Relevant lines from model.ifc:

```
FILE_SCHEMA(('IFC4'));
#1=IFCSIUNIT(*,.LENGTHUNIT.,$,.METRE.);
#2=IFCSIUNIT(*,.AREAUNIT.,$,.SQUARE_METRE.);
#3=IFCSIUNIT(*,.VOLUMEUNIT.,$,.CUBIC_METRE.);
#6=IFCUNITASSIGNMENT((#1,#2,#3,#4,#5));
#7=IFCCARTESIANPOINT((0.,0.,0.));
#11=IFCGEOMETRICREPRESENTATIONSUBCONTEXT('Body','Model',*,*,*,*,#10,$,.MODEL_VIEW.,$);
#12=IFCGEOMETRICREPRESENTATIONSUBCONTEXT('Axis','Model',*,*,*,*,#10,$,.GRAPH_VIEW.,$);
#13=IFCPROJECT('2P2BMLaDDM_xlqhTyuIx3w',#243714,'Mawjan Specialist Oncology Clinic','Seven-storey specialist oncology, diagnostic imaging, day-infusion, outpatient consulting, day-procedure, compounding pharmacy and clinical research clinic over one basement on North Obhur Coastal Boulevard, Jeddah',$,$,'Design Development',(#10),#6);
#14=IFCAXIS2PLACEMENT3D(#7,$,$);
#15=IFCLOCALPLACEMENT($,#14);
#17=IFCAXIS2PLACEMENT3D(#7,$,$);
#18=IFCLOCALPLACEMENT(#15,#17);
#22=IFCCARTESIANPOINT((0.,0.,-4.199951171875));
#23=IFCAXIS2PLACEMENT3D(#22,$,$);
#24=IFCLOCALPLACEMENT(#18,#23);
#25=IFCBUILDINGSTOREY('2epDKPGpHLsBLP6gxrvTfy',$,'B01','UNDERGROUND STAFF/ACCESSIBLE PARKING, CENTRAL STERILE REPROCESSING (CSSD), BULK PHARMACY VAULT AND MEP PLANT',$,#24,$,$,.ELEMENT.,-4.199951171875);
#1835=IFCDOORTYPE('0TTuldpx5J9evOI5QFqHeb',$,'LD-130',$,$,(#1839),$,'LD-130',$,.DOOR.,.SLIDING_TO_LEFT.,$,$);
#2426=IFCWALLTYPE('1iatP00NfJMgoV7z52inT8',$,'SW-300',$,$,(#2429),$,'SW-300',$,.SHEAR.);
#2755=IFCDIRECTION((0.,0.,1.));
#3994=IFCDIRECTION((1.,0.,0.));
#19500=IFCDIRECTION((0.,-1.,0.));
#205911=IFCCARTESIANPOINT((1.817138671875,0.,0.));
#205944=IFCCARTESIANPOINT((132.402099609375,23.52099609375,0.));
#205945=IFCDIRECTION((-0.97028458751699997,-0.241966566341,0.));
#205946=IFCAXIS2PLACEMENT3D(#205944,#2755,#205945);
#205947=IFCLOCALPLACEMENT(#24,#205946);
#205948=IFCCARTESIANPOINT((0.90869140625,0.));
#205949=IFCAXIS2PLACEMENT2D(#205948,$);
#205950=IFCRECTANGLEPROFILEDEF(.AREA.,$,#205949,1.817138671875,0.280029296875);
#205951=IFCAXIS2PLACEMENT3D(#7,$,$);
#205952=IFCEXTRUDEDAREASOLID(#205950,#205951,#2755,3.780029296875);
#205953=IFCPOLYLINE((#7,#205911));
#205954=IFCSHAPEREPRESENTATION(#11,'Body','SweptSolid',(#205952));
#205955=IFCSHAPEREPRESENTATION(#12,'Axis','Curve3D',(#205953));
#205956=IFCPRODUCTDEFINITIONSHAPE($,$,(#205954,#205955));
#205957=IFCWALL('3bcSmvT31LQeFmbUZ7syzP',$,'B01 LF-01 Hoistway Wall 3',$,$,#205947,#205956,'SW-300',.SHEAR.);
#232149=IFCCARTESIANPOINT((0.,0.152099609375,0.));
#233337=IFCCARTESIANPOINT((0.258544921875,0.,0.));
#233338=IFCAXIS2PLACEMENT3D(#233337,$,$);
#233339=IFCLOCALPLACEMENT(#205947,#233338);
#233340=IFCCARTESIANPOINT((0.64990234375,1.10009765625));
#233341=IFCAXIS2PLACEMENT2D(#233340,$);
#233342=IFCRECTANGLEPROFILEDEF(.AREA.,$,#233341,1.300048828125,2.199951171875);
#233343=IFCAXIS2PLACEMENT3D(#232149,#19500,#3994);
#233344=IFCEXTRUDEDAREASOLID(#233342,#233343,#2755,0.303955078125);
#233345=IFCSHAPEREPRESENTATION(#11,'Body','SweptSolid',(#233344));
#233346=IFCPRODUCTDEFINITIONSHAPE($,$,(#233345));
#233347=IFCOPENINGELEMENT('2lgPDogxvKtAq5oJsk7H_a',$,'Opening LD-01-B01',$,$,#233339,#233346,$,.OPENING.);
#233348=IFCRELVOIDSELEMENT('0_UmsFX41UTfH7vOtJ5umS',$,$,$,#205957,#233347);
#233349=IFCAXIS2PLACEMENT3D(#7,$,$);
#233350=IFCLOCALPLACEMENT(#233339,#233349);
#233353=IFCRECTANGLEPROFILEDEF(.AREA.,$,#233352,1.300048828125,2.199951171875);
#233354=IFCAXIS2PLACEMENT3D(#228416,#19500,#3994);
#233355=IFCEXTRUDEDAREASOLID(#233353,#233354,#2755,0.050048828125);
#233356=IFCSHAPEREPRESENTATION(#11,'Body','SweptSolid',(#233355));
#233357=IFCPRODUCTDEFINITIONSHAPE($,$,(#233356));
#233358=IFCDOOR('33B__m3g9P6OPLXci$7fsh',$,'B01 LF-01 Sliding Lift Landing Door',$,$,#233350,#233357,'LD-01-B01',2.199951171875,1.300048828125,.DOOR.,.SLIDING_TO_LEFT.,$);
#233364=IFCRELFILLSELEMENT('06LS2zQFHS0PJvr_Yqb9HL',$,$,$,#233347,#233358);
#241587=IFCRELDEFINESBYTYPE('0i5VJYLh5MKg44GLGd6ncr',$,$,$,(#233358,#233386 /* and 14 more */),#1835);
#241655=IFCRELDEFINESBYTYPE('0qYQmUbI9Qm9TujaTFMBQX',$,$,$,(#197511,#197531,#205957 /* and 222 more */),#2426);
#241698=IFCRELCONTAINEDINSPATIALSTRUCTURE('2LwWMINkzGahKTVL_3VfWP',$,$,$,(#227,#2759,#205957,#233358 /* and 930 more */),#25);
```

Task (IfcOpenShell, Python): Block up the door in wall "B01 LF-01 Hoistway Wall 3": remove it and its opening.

```python
import ifcopenshell
import ifcopenshell.api.feature
import ifcopenshell.api.root
import ifcopenshell.geom
import ifcopenshell.util.shape

model = ifcopenshell.open("model.ifc")
settings = ifcopenshell.geom.settings()


def volume(element):
    """Net volume in cubic metres, openings subtracted."""
    shape = ifcopenshell.geom.create_shape(settings, element)
    return ifcopenshell.util.shape.get_volume(shape.geometry)


door = model.by_guid("33B__m3g9P6OPLXci$7fsh")
opening = door.FillsVoids[0].RelatingOpeningElement
wall = opening.VoidsElements[0].RelatingBuildingElement
before = volume(wall)

ifcopenshell.api.root.remove_product(model, product=door)
ifcopenshell.api.feature.remove_feature(model, feature=opening)

after = volume(wall)

print(f"wall volume {before:.3f} -> {after:.3f} m3")

model.write("model_rev.ifc")
```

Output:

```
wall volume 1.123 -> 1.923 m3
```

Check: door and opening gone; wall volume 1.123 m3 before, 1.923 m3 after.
